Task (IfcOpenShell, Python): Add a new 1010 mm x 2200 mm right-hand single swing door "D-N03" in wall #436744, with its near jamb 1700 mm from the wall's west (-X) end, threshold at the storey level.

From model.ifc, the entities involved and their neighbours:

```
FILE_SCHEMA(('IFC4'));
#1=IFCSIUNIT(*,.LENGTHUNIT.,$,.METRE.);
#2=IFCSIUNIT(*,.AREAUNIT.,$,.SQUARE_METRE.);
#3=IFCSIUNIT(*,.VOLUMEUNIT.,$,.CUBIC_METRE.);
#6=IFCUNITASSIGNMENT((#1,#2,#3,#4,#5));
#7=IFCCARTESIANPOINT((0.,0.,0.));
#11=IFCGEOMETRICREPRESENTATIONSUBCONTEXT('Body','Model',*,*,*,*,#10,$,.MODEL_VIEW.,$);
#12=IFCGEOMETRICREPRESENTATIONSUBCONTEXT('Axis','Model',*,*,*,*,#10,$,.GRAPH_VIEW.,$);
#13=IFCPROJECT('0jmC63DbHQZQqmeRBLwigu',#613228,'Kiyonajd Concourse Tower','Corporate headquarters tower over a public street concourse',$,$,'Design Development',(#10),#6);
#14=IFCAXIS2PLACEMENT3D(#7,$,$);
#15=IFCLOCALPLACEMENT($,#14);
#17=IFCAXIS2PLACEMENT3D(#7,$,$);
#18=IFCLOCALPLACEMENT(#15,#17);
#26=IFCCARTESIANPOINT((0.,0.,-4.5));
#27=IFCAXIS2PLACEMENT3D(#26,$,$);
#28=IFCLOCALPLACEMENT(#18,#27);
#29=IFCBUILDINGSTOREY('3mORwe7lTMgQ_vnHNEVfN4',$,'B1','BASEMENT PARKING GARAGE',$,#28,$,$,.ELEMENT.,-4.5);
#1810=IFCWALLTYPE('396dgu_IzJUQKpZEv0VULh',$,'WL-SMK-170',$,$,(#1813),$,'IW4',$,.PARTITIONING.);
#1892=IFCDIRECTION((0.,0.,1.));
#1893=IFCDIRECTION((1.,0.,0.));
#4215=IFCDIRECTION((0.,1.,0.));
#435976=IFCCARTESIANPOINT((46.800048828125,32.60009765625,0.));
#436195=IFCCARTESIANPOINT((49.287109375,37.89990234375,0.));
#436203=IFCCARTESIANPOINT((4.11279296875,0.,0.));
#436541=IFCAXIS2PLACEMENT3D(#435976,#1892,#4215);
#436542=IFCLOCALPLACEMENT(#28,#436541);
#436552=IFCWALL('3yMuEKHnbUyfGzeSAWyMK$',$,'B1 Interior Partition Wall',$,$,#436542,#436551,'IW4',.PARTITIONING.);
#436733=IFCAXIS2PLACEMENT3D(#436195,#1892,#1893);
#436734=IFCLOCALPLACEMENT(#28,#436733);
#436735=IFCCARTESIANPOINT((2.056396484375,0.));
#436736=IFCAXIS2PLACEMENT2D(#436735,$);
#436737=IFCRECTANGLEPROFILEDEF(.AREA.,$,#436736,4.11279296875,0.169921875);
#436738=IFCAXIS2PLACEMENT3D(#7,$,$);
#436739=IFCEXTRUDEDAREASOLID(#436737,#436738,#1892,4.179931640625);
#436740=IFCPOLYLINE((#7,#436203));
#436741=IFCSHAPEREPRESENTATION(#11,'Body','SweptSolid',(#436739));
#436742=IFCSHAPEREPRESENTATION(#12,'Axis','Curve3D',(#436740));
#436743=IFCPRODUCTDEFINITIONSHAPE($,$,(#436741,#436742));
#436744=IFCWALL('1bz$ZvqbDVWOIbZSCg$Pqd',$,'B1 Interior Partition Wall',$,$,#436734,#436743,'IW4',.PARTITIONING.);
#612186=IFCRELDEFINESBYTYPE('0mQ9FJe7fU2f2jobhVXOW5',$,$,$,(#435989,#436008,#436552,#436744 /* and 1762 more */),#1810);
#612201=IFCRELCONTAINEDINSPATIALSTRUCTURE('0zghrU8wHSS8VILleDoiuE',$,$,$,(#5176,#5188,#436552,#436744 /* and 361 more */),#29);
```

```python
import numpy as np
import ifcopenshell
import ifcopenshell.api.feature
import ifcopenshell.api.geometry
import ifcopenshell.api.root
import ifcopenshell.api.spatial
import ifcopenshell.geom
import ifcopenshell.util.element
import ifcopenshell.util.placement
import ifcopenshell.util.representation
import ifcopenshell.util.shape
import ifcopenshell.util.unit

model = ifcopenshell.open("model.ifc")
unit_scale = ifcopenshell.util.unit.calculate_unit_scale(model)
settings = ifcopenshell.geom.settings()


def volume(element):
    """Net volume in cubic metres, openings subtracted."""
    shape = ifcopenshell.geom.create_shape(settings, element)
    return ifcopenshell.util.shape.get_volume(shape.geometry)


wall = model.by_guid("1bz$ZvqbDVWOIbZSCg$Pqd")
storey = ifcopenshell.util.element.get_container(wall, ifc_class="IfcBuildingStorey")
context = ifcopenshell.util.representation.get_context(model, "Model", "Body", "MODEL_VIEW")
before = volume(wall)

width, height, from_end, sill = 1.01, 2.2, 1.7, 0.0  # metres

# The wall runs along its own X axis, and the end named is its -X end.
wall_shape = ifcopenshell.geom.create_shape(settings, wall)
x, y, z = ifcopenshell.util.shape.get_vertices(wall_shape.geometry).T
start = x.min() + from_end
face, thickness = float(y.min()), float(y.max() - y.min())
wall_matrix = ifcopenshell.util.placement.get_local_placement(wall.ObjectPlacement)
level = ifcopenshell.util.placement.get_local_placement(storey.ObjectPlacement)[2, 3]


def in_wall(x, y):
    """Placement at x, y metres in the wall's axes, at sill height."""
    matrix = wall_matrix.copy()
    matrix[:, 3] = wall_matrix @ np.array([x / unit_scale, y / unit_scale, 0.0, 1.0])
    matrix[2, 3] = level + sill / unit_scale
    return matrix


# Opening: a box that overshoots both wall faces by 50 mm.
opening = ifcopenshell.api.root.create_entity(model, ifc_class="IfcOpeningElement", predefined_type="OPENING")
box = ifcopenshell.api.geometry.add_wall_representation(
    model, context=context, length=width, height=height, thickness=thickness + 0.1
)
ifcopenshell.api.geometry.assign_representation(model, product=opening, representation=box)
ifcopenshell.api.geometry.edit_object_placement(model, product=opening, matrix=in_wall(start, face - 0.05), is_si=False)
ifcopenshell.api.feature.add_feature(model, feature=opening, element=wall)

door = ifcopenshell.api.root.create_entity(model, ifc_class="IfcDoor", name="D-N03", predefined_type="DOOR")
door.OverallWidth, door.OverallHeight = width / unit_scale, height / unit_scale
door.OperationType = "SINGLE_SWING_RIGHT"
body = ifcopenshell.api.geometry.add_door_representation(
    model,
    context=context,
    overall_width=door.OverallWidth,
    overall_height=door.OverallHeight,
    operation_type="SINGLE_SWING_RIGHT",
    lining_properties={"LiningDepth": thickness / unit_scale, "ThresholdDepth": thickness / unit_scale},
)
ifcopenshell.api.geometry.assign_representation(model, product=door, representation=body)
ifcopenshell.api.spatial.assign_container(model, products=[door], relating_structure=storey)
ifcopenshell.api.feature.add_filling(model, opening=opening, element=door)

# The lining spans the wall, so the door starts at the wall face.
ifcopenshell.api.geometry.edit_object_placement(model, product=door, matrix=in_wall(start, face), is_si=False)

after = volume(wall)

print(f"wall volume {before:.3f} -> {after:.3f} m3")

model.write("model-out.ifc")
```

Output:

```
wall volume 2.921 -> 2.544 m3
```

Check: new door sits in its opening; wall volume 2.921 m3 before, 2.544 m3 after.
